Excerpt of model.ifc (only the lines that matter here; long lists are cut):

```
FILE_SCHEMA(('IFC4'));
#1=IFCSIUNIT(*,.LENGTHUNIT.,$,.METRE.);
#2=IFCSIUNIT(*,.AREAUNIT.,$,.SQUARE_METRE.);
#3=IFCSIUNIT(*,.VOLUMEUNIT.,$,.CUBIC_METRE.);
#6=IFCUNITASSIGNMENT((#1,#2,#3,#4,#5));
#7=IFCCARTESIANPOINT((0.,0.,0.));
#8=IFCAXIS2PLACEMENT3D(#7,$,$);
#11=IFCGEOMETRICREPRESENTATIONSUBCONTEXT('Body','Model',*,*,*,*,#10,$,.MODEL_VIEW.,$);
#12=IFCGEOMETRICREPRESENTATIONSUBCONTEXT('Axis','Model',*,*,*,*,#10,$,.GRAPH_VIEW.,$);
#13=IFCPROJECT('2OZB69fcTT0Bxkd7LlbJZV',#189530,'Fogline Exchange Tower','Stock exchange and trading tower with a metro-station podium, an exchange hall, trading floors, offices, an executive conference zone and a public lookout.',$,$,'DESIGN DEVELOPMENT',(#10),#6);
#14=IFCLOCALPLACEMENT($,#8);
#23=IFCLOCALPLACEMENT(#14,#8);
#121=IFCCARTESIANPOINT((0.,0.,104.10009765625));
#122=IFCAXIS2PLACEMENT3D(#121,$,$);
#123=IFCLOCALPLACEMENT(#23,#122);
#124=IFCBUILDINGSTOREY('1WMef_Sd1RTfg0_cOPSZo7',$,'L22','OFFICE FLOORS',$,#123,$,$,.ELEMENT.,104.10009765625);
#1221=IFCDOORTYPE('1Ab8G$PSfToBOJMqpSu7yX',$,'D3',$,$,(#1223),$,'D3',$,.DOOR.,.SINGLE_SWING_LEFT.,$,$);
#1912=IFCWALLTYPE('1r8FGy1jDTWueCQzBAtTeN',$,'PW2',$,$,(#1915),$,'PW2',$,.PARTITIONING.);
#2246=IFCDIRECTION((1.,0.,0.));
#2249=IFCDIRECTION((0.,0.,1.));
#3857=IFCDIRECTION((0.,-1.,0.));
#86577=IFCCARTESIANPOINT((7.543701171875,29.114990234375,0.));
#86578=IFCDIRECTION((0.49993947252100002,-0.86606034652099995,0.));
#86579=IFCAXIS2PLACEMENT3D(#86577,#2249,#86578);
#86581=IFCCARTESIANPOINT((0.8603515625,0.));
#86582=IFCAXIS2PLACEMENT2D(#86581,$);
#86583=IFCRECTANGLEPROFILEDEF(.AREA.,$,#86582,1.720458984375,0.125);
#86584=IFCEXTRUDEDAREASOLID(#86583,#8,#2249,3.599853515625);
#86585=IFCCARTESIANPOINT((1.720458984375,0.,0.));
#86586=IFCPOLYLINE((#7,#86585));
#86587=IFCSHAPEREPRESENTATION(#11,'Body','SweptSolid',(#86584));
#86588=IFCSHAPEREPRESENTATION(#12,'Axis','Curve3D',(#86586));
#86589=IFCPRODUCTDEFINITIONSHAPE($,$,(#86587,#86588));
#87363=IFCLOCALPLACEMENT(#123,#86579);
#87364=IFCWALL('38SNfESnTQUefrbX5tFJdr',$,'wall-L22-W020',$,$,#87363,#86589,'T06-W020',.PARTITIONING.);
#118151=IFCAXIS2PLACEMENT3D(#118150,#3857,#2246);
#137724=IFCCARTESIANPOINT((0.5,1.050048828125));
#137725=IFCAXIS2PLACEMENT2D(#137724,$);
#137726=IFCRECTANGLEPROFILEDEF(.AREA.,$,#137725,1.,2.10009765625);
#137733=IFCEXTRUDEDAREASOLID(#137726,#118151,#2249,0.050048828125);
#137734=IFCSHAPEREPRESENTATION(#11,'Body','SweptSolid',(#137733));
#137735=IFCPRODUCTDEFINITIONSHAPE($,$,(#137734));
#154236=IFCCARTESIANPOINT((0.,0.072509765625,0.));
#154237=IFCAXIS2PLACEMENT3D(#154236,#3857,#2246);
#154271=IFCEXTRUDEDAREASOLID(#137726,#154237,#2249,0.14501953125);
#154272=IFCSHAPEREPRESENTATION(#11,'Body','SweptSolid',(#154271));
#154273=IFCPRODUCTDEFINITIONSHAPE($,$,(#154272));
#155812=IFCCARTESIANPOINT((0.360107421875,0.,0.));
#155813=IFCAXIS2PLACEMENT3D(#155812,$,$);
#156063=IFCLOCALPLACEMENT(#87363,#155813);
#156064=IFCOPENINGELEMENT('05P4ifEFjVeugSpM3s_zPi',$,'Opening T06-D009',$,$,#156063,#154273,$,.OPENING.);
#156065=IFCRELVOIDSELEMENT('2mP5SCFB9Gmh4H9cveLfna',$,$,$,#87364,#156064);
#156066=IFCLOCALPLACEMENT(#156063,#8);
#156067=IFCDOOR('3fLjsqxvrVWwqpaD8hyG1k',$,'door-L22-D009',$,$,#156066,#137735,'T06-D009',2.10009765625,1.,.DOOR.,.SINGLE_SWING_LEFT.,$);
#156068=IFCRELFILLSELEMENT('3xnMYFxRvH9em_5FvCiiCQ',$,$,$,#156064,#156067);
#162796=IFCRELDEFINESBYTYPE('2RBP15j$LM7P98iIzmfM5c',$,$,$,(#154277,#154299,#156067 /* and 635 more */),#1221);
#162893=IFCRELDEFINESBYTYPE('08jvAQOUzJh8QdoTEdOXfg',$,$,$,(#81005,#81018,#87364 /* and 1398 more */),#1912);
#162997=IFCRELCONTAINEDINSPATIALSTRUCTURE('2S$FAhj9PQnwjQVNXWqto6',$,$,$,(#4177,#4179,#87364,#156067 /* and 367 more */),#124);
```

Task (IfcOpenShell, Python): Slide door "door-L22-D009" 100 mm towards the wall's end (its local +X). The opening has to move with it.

```python
import ifcopenshell
import ifcopenshell.api.geometry
import ifcopenshell.util.placement
import ifcopenshell.util.unit

model = ifcopenshell.open("model.ifc")
unit_scale = ifcopenshell.util.unit.calculate_unit_scale(model)

door = model.by_id(156067)
opening = door.FillsVoids[0].RelatingOpeningElement
wall = opening.VoidsElements[0].RelatingBuildingElement

wall_matrix = ifcopenshell.util.placement.get_local_placement(wall.ObjectPlacement)
shift = wall_matrix[:3, 0] * 0.1 / unit_scale
before = ifcopenshell.util.placement.get_local_placement(door.ObjectPlacement)[:3, 3].copy()

# The door is placed relative to its opening, so it follows when the opening moves.
matrix = ifcopenshell.util.placement.get_local_placement(opening.ObjectPlacement)
matrix[:3, 3] += shift
ifcopenshell.api.geometry.edit_object_placement(
    model, product=opening, matrix=matrix, is_si=False, should_transform_children=True
)

after = ifcopenshell.util.placement.get_local_placement(door.ObjectPlacement)[:3, 3]
print("door moved by", (after - before).round(3) + 0.0)

model.write("model_updated.ifc")
```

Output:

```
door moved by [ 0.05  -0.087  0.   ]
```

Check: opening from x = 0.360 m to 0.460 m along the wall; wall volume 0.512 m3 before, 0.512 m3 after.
